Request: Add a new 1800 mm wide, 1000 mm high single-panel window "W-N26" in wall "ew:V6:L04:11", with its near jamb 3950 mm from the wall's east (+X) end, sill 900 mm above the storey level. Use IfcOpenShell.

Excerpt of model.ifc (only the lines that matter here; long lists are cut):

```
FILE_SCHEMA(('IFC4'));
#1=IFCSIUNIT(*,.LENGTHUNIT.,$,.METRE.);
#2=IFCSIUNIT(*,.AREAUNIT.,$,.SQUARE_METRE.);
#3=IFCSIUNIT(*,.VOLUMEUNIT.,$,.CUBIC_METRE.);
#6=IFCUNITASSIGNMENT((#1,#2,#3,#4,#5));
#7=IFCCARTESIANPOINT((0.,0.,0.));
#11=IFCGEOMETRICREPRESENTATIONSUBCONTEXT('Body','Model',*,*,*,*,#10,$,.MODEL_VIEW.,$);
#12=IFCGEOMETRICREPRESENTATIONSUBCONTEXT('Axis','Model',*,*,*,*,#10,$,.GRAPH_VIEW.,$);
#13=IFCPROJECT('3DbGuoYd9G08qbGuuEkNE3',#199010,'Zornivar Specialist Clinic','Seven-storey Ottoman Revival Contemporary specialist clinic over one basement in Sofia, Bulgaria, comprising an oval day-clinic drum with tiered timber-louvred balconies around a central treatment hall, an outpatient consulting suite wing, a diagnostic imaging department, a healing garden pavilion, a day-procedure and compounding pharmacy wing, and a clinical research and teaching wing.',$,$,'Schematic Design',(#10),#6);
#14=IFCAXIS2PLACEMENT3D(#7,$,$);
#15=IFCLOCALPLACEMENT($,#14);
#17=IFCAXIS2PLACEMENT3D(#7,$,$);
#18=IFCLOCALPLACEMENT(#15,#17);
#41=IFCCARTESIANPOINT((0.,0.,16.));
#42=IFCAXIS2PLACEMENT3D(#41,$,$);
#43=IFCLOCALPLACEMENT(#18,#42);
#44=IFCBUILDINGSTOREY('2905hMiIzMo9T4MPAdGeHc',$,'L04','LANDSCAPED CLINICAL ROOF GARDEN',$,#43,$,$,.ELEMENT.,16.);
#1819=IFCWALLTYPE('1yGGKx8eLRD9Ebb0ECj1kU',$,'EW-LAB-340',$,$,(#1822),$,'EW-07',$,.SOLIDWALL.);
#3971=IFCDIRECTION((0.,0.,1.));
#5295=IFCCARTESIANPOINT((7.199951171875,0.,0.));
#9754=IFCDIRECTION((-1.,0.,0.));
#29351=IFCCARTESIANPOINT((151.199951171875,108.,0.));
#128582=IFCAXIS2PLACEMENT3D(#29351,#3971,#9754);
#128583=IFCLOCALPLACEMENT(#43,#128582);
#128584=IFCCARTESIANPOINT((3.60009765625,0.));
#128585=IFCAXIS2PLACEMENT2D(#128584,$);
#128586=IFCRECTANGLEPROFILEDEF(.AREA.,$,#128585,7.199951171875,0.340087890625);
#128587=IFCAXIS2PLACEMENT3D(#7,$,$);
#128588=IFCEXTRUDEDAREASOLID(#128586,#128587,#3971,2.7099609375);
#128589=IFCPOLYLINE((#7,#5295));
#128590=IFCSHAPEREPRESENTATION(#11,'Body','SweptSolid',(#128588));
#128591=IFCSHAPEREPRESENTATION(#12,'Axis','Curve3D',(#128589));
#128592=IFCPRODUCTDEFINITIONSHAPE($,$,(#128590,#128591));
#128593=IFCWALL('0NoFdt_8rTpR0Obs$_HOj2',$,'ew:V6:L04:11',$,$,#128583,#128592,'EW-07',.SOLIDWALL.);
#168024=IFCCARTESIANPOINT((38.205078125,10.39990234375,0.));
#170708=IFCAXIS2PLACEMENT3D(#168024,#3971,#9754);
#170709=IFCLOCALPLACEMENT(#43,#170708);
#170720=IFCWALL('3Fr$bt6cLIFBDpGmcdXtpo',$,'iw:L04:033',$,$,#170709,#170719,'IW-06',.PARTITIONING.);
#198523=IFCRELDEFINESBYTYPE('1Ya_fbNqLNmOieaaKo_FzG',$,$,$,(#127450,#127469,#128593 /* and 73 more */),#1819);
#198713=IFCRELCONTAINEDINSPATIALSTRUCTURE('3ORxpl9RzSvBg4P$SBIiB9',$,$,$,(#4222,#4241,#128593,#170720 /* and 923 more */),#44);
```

```python
import numpy as np
import ifcopenshell
import ifcopenshell.api.feature
import ifcopenshell.api.geometry
import ifcopenshell.api.root
import ifcopenshell.api.spatial
import ifcopenshell.geom
import ifcopenshell.util.element
import ifcopenshell.util.placement
import ifcopenshell.util.representation
import ifcopenshell.util.shape
import ifcopenshell.util.unit

model = ifcopenshell.open("model.ifc")
unit_scale = ifcopenshell.util.unit.calculate_unit_scale(model)
settings = ifcopenshell.geom.settings()


def volume(element):
    """Net volume in cubic metres, openings subtracted."""
    shape = ifcopenshell.geom.create_shape(settings, element)
    return ifcopenshell.util.shape.get_volume(shape.geometry)


wall = model.by_guid("0NoFdt_8rTpR0Obs$_HOj2")
storey = ifcopenshell.util.element.get_container(wall, ifc_class="IfcBuildingStorey")
context = ifcopenshell.util.representation.get_context(model, "Model", "Body", "MODEL_VIEW")
before = volume(wall)

width, height, from_end, sill = 1.8, 1, 3.95, 0.9  # metres

# The wall runs along its own X axis, and the end named is its -X end.
wall_shape = ifcopenshell.geom.create_shape(settings, wall)
x, y, z = ifcopenshell.util.shape.get_vertices(wall_shape.geometry).T
start = x.min() + from_end
face, thickness = float(y.min()), float(y.max() - y.min())
wall_matrix = ifcopenshell.util.placement.get_local_placement(wall.ObjectPlacement)
level = ifcopenshell.util.placement.get_local_placement(storey.ObjectPlacement)[2, 3]


def in_wall(x, y):
    """Placement at x, y metres in the wall's axes, at sill height."""
    matrix = wall_matrix.copy()
    matrix[:, 3] = wall_matrix @ np.array([x / unit_scale, y / unit_scale, 0.0, 1.0])
    matrix[2, 3] = level + sill / unit_scale
    return matrix


# Opening: a box that overshoots both wall faces by 50 mm.
opening = ifcopenshell.api.root.create_entity(model, ifc_class="IfcOpeningElement", predefined_type="OPENING")
box = ifcopenshell.api.geometry.add_wall_representation(
    model, context=context, length=width, height=height, thickness=thickness + 0.1
)
ifcopenshell.api.geometry.assign_representation(model, product=opening, representation=box)
ifcopenshell.api.geometry.edit_object_placement(model, product=opening, matrix=in_wall(start, face - 0.05), is_si=False)
ifcopenshell.api.feature.add_feature(model, feature=opening, element=wall)

window = ifcopenshell.api.root.create_entity(model, ifc_class="IfcWindow", name="W-N26", predefined_type="WINDOW")
window.OverallWidth, window.OverallHeight = width / unit_scale, height / unit_scale
window.PartitioningType = "SINGLE_PANEL"
body = ifcopenshell.api.geometry.add_window_representation(
    model,
    context=context,
    overall_width=window.OverallWidth,
    overall_height=window.OverallHeight,
    partition_type="SINGLE_PANEL",
)
ifcopenshell.api.geometry.assign_representation(model, product=window, representation=body)
ifcopenshell.api.spatial.assign_container(model, products=[window], relating_structure=storey)
ifcopenshell.api.feature.add_filling(model, opening=opening, element=window)

# Centre the window in the wall's thickness.
ifcopenshell.api.geometry.edit_object_placement(model, product=window, matrix=in_wall(start, face), is_si=False)
window_shape = ifcopenshell.geom.create_shape(settings, window)
depth = ifcopenshell.util.shape.get_vertices(window_shape.geometry)[:, 1]
offset = face + thickness / 2 - (depth.min() + depth.max()) / 2
ifcopenshell.api.geometry.edit_object_placement(model, product=window, matrix=in_wall(start, offset), is_si=False)

after = volume(wall)

print(f"wall volume {before:.3f} -> {after:.3f} m3")

model.write("model_rev.ifc")
```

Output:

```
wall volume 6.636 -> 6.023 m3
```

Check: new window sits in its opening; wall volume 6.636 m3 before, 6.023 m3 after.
